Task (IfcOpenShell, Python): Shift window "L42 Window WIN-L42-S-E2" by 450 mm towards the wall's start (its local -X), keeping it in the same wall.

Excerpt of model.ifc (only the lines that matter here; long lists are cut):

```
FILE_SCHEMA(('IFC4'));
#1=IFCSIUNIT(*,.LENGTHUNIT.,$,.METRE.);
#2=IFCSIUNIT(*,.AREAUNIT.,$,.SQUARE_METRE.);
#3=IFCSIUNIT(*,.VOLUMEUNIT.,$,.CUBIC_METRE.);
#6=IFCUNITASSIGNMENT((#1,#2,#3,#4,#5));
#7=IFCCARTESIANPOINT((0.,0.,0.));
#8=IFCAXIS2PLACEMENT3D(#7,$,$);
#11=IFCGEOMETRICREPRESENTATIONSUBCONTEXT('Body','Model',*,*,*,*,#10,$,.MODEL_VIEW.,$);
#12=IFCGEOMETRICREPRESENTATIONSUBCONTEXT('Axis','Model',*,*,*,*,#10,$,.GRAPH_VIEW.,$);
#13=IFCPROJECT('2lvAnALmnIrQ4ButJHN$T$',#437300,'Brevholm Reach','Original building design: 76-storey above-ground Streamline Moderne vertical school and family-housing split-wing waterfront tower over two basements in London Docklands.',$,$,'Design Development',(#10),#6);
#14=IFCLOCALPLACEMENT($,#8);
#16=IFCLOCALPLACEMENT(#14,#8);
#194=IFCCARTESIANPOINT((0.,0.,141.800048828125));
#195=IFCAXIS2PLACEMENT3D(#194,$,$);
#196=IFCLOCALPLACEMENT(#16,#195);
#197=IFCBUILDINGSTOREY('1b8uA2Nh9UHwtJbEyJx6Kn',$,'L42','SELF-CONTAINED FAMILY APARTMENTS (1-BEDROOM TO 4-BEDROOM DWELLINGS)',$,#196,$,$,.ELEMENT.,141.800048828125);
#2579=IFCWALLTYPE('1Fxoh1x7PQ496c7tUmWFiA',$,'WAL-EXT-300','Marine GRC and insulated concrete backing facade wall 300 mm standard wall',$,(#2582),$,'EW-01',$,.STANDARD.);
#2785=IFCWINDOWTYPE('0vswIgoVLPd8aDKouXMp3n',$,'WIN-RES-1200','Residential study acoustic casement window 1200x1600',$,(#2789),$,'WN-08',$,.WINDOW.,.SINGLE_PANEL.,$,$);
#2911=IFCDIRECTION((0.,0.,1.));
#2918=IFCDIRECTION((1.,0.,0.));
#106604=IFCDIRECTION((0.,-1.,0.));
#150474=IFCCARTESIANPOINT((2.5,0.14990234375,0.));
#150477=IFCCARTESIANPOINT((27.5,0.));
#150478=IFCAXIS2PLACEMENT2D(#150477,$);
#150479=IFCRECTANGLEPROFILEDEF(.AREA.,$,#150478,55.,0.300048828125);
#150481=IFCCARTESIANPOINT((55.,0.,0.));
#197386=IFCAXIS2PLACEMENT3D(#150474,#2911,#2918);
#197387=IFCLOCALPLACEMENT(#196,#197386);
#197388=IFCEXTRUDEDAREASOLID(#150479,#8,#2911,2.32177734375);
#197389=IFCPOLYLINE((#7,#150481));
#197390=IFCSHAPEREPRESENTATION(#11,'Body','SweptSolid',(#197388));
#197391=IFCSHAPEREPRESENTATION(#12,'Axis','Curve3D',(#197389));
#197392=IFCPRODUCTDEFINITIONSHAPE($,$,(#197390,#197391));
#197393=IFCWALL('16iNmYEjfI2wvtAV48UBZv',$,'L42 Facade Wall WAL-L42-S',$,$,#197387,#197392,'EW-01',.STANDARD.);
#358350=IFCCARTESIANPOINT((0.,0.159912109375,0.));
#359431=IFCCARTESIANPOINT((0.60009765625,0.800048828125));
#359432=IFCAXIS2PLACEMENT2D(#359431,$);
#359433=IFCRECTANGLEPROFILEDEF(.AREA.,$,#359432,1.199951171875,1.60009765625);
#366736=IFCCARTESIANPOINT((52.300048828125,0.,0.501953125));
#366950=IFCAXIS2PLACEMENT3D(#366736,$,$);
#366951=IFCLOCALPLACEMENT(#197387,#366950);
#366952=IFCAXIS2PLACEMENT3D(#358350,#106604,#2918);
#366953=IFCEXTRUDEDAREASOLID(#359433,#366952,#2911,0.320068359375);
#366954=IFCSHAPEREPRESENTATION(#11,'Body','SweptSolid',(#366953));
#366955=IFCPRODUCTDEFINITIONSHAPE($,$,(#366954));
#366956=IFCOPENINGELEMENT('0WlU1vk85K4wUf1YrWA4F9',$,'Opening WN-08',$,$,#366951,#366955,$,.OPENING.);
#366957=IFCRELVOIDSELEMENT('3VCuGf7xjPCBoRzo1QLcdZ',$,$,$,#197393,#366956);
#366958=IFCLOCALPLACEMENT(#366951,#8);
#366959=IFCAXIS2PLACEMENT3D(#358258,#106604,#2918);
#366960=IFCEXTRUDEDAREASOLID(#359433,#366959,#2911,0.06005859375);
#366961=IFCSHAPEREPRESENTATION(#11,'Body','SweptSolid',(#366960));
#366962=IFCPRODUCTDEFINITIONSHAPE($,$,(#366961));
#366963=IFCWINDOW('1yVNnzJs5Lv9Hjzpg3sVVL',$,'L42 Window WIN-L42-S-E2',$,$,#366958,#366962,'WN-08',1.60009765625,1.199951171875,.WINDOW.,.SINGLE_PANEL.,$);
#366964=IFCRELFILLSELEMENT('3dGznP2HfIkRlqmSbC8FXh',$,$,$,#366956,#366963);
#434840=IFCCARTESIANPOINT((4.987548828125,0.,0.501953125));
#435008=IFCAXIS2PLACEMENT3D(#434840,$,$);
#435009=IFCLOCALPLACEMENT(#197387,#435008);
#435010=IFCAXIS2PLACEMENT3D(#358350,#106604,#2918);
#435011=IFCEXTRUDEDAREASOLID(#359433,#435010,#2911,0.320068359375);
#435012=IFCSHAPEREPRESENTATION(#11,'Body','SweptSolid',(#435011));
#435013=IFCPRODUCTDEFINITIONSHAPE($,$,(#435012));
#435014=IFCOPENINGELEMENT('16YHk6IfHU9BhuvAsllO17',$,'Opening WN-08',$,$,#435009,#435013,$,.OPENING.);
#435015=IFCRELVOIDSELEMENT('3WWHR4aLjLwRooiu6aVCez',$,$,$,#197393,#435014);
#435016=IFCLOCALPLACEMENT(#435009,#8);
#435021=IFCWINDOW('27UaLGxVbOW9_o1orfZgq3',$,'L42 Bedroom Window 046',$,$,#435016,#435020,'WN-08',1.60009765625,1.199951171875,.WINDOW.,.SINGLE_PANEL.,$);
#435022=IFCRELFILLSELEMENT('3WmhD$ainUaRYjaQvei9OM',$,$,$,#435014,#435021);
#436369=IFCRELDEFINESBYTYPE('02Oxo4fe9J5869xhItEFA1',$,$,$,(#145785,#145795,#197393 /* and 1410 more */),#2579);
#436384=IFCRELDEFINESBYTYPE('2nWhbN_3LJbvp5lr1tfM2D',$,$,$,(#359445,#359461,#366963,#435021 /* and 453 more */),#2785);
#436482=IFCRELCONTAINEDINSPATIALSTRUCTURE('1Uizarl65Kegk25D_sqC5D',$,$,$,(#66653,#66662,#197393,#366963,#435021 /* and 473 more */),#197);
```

```python
import ifcopenshell
import ifcopenshell.api.geometry
import ifcopenshell.util.placement
import ifcopenshell.util.unit

model = ifcopenshell.open("model.ifc")
unit_scale = ifcopenshell.util.unit.calculate_unit_scale(model)

window = model.by_guid("1yVNnzJs5Lv9Hjzpg3sVVL")
opening = window.FillsVoids[0].RelatingOpeningElement
wall = opening.VoidsElements[0].RelatingBuildingElement

wall_matrix = ifcopenshell.util.placement.get_local_placement(wall.ObjectPlacement)
shift = wall_matrix[:3, 0] * -0.45 / unit_scale
before = ifcopenshell.util.placement.get_local_placement(window.ObjectPlacement)[:3, 3].copy()

# The window is placed relative to its opening, so it follows when the opening moves.
matrix = ifcopenshell.util.placement.get_local_placement(opening.ObjectPlacement)
matrix[:3, 3] += shift
ifcopenshell.api.geometry.edit_object_placement(
    model, product=opening, matrix=matrix, is_si=False, should_transform_children=True
)

after = ifcopenshell.util.placement.get_local_placement(window.ObjectPlacement)[:3, 3]
print("window moved by", (after - before).round(3) + 0.0)

model.write("model_v2.ifc")
```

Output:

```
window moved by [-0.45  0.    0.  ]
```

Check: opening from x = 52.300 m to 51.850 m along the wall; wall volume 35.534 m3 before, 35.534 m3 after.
